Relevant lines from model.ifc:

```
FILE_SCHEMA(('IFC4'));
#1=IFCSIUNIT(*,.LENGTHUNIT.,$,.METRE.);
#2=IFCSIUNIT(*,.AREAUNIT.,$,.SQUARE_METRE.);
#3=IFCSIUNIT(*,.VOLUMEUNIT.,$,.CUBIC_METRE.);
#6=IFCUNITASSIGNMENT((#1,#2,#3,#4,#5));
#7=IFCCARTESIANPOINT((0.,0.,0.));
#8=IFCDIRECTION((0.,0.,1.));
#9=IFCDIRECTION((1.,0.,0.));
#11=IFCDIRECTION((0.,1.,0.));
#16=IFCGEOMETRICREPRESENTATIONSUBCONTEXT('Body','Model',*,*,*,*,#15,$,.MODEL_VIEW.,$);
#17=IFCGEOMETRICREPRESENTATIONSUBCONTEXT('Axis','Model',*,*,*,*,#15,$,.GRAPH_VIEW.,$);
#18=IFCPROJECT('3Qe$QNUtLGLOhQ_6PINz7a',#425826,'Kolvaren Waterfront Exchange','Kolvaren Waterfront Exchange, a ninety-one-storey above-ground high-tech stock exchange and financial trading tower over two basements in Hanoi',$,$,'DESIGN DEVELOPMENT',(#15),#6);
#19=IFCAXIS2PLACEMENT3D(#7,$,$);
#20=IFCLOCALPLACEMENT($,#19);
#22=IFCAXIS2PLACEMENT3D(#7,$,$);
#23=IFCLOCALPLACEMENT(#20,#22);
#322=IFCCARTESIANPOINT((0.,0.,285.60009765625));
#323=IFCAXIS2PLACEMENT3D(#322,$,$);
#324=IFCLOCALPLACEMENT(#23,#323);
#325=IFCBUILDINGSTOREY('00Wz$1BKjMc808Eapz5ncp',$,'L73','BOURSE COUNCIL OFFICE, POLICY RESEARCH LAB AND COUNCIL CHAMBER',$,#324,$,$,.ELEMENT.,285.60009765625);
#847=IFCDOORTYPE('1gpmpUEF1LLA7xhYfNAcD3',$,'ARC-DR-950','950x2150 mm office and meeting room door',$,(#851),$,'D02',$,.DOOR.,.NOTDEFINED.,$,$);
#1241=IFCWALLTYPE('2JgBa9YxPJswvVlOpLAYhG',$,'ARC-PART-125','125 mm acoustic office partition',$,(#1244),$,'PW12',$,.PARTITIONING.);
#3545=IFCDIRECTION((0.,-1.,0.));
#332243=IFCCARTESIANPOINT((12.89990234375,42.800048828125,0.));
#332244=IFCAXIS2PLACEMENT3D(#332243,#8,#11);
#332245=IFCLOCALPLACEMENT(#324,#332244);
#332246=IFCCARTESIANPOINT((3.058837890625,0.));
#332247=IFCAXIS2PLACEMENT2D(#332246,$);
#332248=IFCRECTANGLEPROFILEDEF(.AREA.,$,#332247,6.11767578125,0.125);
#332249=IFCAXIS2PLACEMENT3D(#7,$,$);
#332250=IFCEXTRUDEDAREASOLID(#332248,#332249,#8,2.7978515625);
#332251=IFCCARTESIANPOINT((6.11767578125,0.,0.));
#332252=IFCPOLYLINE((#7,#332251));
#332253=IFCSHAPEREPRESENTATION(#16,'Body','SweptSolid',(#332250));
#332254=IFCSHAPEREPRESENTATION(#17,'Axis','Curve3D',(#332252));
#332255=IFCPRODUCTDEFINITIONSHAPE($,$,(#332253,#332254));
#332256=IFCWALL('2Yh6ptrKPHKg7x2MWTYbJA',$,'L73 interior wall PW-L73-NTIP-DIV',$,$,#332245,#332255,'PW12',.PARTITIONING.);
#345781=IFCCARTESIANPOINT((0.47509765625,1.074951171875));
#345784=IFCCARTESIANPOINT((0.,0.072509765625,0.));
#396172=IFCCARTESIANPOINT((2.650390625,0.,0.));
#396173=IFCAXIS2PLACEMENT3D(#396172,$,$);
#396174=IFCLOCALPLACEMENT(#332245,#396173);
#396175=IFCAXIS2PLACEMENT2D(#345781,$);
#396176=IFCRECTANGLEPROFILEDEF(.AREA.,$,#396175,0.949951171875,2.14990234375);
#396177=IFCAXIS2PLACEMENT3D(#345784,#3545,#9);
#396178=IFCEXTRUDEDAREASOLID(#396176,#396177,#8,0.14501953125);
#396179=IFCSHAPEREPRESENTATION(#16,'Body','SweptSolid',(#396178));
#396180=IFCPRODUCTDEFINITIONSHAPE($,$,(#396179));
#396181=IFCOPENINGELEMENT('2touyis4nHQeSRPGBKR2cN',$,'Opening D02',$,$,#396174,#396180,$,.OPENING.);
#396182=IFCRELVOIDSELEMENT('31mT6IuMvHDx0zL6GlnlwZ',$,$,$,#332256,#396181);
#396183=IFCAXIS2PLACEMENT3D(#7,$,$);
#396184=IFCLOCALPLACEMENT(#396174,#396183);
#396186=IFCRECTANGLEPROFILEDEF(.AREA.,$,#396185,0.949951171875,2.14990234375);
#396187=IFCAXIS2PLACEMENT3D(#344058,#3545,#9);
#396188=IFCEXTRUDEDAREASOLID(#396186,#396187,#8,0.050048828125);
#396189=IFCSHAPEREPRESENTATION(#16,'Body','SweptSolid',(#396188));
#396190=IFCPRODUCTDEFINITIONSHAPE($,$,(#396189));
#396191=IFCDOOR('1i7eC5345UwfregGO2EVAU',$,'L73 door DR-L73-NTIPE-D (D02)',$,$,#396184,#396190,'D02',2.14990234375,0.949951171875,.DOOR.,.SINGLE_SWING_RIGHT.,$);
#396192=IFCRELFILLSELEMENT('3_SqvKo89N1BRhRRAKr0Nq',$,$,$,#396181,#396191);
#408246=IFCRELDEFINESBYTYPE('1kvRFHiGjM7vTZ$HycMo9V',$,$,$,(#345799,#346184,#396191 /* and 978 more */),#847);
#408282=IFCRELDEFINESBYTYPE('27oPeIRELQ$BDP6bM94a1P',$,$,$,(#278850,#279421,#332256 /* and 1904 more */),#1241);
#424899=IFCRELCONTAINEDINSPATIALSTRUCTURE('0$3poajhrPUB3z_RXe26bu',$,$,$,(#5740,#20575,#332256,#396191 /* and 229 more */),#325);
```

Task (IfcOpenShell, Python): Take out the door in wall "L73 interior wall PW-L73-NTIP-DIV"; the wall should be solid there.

```python
import ifcopenshell
import ifcopenshell.api.feature
import ifcopenshell.api.root
import ifcopenshell.geom
import ifcopenshell.util.shape

model = ifcopenshell.open("model.ifc")
settings = ifcopenshell.geom.settings()


def volume(element):
    """Net volume in cubic metres, openings subtracted."""
    shape = ifcopenshell.geom.create_shape(settings, element)
    return ifcopenshell.util.shape.get_volume(shape.geometry)


door = model.by_guid("1i7eC5345UwfregGO2EVAU")
opening = door.FillsVoids[0].RelatingOpeningElement
wall = opening.VoidsElements[0].RelatingBuildingElement
before = volume(wall)

ifcopenshell.api.root.remove_product(model, product=door)
ifcopenshell.api.feature.remove_feature(model, feature=opening)

after = volume(wall)

print(f"wall volume {before:.3f} -> {after:.3f} m3")

model.write("model_rev.ifc")
```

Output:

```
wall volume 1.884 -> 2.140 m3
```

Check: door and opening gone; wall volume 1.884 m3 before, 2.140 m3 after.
